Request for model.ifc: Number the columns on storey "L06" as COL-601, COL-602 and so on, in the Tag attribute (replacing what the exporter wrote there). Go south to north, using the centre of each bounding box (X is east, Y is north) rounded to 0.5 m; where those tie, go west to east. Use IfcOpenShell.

First a look at what the model holds.

```python
import ifcopenshell
import ifcopenshell.util.element
import ifcopenshell.util.placement

model = ifcopenshell.open("model.ifc")
print(model.schema)
storey = next(s for s in model.by_type("IfcBuildingStorey") if s.Name == "L06")
columns = [e for e in ifcopenshell.util.element.get_decomposition(storey) if e.is_a("IfcColumn")]
for e in sorted(columns, key=lambda e: e.id()):
    origin = ifcopenshell.util.placement.get_local_placement(e.ObjectPlacement)[:3, 3]
    print(e.id(), e.Tag, e.Name, origin.round(2) + 0.0, sep=" | ")
```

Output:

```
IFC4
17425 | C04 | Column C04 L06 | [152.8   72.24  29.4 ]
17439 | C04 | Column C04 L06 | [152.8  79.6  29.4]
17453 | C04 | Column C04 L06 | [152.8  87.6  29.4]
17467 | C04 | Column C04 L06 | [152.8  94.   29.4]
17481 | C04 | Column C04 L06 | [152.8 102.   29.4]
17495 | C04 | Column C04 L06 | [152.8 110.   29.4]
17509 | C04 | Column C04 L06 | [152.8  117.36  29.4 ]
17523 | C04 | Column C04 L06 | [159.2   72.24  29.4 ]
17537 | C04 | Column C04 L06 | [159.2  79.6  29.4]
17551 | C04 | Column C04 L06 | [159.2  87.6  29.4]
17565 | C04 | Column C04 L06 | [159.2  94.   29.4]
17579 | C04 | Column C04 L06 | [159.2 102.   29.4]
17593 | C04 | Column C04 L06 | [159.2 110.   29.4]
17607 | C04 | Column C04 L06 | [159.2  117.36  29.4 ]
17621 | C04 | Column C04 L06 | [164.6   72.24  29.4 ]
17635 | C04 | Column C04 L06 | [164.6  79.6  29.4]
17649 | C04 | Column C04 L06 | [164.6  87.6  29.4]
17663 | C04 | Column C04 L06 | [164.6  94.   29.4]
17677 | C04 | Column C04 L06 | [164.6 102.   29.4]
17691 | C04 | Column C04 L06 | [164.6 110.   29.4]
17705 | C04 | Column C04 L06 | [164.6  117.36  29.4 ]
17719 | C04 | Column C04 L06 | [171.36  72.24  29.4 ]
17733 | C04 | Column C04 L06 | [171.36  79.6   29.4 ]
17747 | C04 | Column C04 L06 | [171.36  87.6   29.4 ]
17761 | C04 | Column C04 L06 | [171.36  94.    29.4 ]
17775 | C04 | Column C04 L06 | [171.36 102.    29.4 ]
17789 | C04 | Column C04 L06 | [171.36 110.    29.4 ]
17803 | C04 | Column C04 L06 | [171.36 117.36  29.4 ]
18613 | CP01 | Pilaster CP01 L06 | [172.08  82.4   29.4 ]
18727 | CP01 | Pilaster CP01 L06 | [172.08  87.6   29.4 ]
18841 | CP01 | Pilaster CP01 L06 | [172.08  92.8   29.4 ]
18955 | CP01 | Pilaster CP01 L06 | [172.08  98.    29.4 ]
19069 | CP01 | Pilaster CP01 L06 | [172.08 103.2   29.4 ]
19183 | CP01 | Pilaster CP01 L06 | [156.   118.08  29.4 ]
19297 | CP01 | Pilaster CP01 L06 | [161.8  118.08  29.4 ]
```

```python
import ifcopenshell
import ifcopenshell.geom
import ifcopenshell.util.element
import ifcopenshell.util.shape

model = ifcopenshell.open("model.ifc")
settings = ifcopenshell.geom.settings()
settings.set("use-world-coords", True)


def centre(element):
    shape = ifcopenshell.geom.create_shape(settings, element)
    return ifcopenshell.util.shape.get_bbox_centroid(shape.geometry)


storey = next(s for s in model.by_type("IfcBuildingStorey") if s.Name == "L06")
columns = [e for e in ifcopenshell.util.element.get_decomposition(storey) if e.is_a("IfcColumn")]

# Insertion points can sit at a corner or the storey origin, so sort by the geometry (in metres).
centres = {e: centre(e) for e in columns}
columns.sort(key=lambda e: (round(centres[e][1] / 0.5), centres[e][0]))

for i, e in enumerate(columns, start=1):
    number = f"COL-6{i:02d}"
    e.Tag = number
    print(e.id(), number)

model.write("model-out.ifc")
```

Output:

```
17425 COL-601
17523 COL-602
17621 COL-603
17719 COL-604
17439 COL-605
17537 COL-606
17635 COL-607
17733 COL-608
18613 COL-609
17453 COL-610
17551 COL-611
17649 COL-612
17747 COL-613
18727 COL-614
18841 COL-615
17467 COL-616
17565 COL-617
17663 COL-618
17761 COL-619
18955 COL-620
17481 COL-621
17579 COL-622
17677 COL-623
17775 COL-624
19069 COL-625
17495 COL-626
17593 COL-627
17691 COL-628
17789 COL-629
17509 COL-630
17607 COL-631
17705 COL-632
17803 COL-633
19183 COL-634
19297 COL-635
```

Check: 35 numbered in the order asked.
